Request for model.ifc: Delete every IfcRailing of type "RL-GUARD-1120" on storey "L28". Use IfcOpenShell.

First a look at what the model holds.

```python
import ifcopenshell
import ifcopenshell.util.element

model = ifcopenshell.open("model.ifc")
print(model.schema)
storey = next(s for s in model.by_type("IfcBuildingStorey") if s.Name == "L28")
railings = [e for e in ifcopenshell.util.element.get_decomposition(storey) if e.is_a("IfcRailing")]
seen = {}
for e in railings:
    element_type = ifcopenshell.util.element.get_type(e)
    name = element_type.Name if element_type not in (None, e) else None
    seen[name] = seen.get(name, 0) + 1
for name, count in sorted(seen.items(), key=str):
    print(count, "x", name)
```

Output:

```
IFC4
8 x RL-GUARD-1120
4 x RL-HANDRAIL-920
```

```python
import ifcopenshell
import ifcopenshell.api.root
import ifcopenshell.util.element

model = ifcopenshell.open("model.ifc")

storey = next(s for s in model.by_type("IfcBuildingStorey") if s.Name == "L28")
railings = [e for e in ifcopenshell.util.element.get_decomposition(storey) if e.is_a("IfcRailing")]
targets = [e for e in railings if (t := ifcopenshell.util.element.get_type(e)) not in (None, e) and t.Name == "RL-GUARD-1120"]

for e in targets:
    ifcopenshell.api.root.remove_product(model, product=e)
print(len(targets), "removed")

model.write("model-out.ifc")
```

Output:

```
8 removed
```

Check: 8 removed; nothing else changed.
